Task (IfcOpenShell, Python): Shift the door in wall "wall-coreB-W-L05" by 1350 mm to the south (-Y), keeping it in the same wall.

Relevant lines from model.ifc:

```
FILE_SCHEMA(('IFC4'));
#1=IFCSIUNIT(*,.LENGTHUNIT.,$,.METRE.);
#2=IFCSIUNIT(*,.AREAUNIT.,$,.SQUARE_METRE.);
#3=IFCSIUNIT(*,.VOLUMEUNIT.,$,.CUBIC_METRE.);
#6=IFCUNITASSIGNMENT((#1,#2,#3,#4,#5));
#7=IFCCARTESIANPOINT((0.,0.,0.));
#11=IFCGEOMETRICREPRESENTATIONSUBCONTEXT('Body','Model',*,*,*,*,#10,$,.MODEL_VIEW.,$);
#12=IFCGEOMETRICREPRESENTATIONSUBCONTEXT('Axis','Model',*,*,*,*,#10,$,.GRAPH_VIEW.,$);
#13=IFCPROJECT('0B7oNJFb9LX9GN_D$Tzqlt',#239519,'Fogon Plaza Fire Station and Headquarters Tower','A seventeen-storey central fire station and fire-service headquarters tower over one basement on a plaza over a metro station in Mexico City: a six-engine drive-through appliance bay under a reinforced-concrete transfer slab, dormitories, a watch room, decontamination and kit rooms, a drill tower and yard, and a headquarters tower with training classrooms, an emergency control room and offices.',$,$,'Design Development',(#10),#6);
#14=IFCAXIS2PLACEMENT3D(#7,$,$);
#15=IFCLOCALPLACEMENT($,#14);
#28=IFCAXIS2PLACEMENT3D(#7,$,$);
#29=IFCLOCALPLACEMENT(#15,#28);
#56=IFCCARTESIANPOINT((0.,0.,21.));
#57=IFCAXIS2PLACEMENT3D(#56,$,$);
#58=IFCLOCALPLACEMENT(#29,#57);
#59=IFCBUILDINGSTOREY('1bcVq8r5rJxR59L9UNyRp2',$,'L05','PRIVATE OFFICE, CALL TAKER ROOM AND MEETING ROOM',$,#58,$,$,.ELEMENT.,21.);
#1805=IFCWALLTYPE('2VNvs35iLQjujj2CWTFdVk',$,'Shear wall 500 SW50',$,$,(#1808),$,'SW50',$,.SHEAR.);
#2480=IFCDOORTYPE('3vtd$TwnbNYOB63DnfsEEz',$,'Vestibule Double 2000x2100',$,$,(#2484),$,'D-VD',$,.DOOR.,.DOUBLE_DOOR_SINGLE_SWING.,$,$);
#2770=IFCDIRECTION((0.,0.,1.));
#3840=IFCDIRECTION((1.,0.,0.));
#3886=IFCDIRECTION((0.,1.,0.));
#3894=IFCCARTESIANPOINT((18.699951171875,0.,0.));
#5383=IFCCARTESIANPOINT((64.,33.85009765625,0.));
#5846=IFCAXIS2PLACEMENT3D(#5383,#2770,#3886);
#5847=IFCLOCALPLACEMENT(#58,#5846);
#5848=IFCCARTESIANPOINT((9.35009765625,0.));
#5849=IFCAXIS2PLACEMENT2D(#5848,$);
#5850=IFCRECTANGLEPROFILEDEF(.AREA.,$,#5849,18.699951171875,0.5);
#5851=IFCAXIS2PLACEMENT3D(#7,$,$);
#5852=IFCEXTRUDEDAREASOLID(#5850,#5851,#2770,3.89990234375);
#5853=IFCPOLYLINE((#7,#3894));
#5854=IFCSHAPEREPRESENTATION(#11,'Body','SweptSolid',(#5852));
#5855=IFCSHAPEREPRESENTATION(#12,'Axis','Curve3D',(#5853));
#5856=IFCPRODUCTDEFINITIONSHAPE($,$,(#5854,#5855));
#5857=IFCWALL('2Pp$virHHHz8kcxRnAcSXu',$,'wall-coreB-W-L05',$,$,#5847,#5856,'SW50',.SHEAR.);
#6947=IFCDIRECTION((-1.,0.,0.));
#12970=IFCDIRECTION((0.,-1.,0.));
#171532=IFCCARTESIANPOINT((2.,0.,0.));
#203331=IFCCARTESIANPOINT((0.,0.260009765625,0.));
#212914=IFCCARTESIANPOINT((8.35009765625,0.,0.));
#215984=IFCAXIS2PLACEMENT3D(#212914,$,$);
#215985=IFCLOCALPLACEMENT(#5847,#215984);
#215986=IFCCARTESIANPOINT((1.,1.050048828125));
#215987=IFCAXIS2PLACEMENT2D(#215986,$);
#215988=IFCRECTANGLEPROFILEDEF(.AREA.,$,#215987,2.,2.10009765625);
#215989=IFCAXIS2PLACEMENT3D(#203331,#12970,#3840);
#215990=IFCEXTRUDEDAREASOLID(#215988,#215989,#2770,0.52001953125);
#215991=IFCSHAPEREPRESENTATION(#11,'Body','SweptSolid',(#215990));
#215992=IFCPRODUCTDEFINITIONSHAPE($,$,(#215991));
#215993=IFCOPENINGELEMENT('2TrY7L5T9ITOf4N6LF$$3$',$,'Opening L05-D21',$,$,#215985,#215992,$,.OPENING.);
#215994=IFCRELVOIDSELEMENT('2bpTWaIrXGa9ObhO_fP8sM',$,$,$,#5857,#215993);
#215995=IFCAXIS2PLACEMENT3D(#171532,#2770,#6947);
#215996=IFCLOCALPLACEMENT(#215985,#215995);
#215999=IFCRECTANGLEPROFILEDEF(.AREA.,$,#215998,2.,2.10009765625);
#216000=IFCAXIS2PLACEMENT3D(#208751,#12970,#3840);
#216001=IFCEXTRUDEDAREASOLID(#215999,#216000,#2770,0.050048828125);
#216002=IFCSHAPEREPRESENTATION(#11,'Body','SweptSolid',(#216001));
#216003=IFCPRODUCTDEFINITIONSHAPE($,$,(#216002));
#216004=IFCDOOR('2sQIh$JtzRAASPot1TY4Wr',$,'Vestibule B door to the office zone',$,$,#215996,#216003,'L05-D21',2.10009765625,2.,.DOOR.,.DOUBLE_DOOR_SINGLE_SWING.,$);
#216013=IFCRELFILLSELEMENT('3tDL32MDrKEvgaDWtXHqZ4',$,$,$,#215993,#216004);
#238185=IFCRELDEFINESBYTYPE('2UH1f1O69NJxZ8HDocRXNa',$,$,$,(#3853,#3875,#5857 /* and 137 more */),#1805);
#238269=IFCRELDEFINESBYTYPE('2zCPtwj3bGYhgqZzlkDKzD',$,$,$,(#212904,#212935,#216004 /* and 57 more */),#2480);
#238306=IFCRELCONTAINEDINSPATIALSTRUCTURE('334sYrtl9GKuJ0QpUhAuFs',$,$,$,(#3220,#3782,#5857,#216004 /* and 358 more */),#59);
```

```python
import ifcopenshell
import ifcopenshell.api.geometry
import ifcopenshell.util.placement

model = ifcopenshell.open("model.ifc")

door = model.by_guid("2sQIh$JtzRAASPot1TY4Wr")
opening = door.FillsVoids[0].RelatingOpeningElement
wall = opening.VoidsElements[0].RelatingBuildingElement

wall_matrix = ifcopenshell.util.placement.get_local_placement(wall.ObjectPlacement)
shift = wall_matrix[:3, 0] * -1.35
before = ifcopenshell.util.placement.get_local_placement(door.ObjectPlacement)[:3, 3].copy()

# The door is placed relative to its opening, so it follows when the opening moves.
matrix = ifcopenshell.util.placement.get_local_placement(opening.ObjectPlacement)
matrix[:3, 3] += shift
ifcopenshell.api.geometry.edit_object_placement(
    model, product=opening, matrix=matrix, is_si=False, should_transform_children=True
)

after = ifcopenshell.util.placement.get_local_placement(door.ObjectPlacement)[:3, 3]
print("door moved by", (after - before).round(3) + 0.0)

model.write("model_updated.ifc")
```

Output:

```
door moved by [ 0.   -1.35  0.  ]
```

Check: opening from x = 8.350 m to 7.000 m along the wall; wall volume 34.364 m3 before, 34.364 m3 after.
